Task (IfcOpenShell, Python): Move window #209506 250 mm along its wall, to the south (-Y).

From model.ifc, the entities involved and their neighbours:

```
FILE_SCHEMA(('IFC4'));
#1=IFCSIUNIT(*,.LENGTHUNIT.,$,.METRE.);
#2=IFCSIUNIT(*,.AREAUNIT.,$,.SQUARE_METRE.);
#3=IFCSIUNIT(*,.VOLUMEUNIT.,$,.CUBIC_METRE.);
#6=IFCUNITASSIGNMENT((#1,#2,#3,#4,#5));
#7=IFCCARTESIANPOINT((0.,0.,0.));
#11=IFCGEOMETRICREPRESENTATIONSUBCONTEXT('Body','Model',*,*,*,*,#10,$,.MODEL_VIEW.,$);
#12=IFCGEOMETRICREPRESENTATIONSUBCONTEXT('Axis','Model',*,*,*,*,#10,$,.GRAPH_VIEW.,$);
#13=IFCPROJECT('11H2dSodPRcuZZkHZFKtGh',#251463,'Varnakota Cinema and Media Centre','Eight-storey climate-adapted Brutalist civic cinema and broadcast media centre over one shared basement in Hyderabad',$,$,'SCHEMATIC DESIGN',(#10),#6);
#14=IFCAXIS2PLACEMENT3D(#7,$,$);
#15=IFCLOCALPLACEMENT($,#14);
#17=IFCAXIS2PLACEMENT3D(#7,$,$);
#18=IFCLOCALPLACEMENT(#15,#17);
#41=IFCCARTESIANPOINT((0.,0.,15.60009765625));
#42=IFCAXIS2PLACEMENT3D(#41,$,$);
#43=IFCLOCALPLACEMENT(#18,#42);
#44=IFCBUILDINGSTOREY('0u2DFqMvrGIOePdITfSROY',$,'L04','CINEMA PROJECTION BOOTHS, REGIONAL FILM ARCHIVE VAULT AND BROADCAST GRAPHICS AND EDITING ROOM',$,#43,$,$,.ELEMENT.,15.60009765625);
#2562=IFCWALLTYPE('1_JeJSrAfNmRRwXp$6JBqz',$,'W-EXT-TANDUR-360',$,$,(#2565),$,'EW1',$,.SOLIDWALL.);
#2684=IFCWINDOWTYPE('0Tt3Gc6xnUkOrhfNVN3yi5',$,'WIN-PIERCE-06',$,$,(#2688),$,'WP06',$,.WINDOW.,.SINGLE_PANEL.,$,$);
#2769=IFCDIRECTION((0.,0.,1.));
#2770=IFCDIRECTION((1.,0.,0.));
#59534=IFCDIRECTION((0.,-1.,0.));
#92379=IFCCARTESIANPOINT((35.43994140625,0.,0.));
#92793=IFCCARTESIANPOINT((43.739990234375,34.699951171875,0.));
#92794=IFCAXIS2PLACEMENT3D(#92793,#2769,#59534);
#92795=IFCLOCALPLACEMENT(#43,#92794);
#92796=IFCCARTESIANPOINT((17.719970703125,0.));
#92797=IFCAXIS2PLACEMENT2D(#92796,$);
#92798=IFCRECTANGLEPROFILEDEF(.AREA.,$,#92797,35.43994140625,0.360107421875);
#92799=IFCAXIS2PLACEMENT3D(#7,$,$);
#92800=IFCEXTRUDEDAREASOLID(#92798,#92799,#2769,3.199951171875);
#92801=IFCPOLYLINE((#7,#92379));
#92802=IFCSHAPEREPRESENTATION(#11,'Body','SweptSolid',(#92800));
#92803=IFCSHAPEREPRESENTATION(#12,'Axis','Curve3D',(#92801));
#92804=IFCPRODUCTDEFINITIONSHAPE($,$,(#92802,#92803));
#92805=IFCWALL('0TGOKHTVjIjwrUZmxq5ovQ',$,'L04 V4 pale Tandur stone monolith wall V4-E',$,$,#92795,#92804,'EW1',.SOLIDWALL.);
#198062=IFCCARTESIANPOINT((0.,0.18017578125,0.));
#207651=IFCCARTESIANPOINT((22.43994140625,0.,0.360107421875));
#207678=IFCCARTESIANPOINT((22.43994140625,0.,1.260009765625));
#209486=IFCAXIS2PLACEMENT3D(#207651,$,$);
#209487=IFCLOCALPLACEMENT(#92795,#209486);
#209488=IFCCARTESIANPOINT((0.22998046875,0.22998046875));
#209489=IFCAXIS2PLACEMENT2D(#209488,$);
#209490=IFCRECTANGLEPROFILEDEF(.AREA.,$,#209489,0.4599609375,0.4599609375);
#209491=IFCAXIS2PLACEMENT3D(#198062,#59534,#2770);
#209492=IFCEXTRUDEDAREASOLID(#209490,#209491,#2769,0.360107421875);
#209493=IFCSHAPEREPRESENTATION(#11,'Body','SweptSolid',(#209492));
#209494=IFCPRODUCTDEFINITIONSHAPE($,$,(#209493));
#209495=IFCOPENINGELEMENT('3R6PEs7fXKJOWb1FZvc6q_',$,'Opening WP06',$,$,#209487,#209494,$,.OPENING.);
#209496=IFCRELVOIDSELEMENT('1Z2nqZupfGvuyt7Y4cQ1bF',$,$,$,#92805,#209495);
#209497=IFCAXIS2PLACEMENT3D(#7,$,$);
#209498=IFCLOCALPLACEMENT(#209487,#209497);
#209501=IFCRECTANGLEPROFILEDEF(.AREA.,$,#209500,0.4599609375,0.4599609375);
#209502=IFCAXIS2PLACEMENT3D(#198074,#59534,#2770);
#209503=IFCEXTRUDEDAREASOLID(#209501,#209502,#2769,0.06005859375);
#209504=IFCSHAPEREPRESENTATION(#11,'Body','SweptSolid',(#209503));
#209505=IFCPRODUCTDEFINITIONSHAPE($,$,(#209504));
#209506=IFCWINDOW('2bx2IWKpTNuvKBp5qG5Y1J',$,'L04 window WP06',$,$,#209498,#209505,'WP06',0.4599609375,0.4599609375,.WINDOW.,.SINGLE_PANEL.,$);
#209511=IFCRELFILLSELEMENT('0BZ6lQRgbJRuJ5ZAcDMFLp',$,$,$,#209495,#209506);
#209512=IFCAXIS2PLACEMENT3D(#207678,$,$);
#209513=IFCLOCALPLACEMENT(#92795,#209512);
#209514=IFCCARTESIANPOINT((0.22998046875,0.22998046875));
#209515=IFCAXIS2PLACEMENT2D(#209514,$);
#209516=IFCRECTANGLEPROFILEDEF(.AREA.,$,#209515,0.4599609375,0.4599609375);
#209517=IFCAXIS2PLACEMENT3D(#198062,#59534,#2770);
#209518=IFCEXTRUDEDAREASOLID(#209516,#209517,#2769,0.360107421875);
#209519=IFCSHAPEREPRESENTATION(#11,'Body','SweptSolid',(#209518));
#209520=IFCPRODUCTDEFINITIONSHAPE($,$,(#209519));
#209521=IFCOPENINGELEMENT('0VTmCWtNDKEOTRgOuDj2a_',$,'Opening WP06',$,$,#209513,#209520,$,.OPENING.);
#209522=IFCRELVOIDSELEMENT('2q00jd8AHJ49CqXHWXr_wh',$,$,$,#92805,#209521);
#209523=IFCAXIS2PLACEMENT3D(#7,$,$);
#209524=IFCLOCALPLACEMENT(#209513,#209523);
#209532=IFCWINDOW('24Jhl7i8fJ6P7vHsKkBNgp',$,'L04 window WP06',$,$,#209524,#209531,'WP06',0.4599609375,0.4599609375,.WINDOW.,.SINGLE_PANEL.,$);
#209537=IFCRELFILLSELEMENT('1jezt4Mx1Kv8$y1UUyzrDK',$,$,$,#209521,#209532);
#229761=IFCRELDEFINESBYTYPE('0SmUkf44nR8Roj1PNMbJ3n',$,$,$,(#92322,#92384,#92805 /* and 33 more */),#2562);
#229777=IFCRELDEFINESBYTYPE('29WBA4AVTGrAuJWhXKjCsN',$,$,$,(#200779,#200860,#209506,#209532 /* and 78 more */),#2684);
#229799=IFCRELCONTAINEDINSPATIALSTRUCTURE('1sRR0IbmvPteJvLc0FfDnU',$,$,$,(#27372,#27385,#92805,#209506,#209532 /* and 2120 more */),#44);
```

```python
import ifcopenshell
import ifcopenshell.api.geometry
import ifcopenshell.util.placement
import ifcopenshell.util.unit

model = ifcopenshell.open("model.ifc")
unit_scale = ifcopenshell.util.unit.calculate_unit_scale(model)

window = model.by_id(209506)
opening = window.FillsVoids[0].RelatingOpeningElement
wall = opening.VoidsElements[0].RelatingBuildingElement

wall_matrix = ifcopenshell.util.placement.get_local_placement(wall.ObjectPlacement)
shift = wall_matrix[:3, 0] * 0.25 / unit_scale
before = ifcopenshell.util.placement.get_local_placement(window.ObjectPlacement)[:3, 3].copy()

# The window is placed relative to its opening, so it follows when the opening moves.
matrix = ifcopenshell.util.placement.get_local_placement(opening.ObjectPlacement)
matrix[:3, 3] += shift
ifcopenshell.api.geometry.edit_object_placement(
    model, product=opening, matrix=matrix, is_si=False, should_transform_children=True
)

after = ifcopenshell.util.placement.get_local_placement(window.ObjectPlacement)[:3, 3]
print("window moved by", (after - before).round(3) + 0.0)

model.write("model_updated.ifc")
```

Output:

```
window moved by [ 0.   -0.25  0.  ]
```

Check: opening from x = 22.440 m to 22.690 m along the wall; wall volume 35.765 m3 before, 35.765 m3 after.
